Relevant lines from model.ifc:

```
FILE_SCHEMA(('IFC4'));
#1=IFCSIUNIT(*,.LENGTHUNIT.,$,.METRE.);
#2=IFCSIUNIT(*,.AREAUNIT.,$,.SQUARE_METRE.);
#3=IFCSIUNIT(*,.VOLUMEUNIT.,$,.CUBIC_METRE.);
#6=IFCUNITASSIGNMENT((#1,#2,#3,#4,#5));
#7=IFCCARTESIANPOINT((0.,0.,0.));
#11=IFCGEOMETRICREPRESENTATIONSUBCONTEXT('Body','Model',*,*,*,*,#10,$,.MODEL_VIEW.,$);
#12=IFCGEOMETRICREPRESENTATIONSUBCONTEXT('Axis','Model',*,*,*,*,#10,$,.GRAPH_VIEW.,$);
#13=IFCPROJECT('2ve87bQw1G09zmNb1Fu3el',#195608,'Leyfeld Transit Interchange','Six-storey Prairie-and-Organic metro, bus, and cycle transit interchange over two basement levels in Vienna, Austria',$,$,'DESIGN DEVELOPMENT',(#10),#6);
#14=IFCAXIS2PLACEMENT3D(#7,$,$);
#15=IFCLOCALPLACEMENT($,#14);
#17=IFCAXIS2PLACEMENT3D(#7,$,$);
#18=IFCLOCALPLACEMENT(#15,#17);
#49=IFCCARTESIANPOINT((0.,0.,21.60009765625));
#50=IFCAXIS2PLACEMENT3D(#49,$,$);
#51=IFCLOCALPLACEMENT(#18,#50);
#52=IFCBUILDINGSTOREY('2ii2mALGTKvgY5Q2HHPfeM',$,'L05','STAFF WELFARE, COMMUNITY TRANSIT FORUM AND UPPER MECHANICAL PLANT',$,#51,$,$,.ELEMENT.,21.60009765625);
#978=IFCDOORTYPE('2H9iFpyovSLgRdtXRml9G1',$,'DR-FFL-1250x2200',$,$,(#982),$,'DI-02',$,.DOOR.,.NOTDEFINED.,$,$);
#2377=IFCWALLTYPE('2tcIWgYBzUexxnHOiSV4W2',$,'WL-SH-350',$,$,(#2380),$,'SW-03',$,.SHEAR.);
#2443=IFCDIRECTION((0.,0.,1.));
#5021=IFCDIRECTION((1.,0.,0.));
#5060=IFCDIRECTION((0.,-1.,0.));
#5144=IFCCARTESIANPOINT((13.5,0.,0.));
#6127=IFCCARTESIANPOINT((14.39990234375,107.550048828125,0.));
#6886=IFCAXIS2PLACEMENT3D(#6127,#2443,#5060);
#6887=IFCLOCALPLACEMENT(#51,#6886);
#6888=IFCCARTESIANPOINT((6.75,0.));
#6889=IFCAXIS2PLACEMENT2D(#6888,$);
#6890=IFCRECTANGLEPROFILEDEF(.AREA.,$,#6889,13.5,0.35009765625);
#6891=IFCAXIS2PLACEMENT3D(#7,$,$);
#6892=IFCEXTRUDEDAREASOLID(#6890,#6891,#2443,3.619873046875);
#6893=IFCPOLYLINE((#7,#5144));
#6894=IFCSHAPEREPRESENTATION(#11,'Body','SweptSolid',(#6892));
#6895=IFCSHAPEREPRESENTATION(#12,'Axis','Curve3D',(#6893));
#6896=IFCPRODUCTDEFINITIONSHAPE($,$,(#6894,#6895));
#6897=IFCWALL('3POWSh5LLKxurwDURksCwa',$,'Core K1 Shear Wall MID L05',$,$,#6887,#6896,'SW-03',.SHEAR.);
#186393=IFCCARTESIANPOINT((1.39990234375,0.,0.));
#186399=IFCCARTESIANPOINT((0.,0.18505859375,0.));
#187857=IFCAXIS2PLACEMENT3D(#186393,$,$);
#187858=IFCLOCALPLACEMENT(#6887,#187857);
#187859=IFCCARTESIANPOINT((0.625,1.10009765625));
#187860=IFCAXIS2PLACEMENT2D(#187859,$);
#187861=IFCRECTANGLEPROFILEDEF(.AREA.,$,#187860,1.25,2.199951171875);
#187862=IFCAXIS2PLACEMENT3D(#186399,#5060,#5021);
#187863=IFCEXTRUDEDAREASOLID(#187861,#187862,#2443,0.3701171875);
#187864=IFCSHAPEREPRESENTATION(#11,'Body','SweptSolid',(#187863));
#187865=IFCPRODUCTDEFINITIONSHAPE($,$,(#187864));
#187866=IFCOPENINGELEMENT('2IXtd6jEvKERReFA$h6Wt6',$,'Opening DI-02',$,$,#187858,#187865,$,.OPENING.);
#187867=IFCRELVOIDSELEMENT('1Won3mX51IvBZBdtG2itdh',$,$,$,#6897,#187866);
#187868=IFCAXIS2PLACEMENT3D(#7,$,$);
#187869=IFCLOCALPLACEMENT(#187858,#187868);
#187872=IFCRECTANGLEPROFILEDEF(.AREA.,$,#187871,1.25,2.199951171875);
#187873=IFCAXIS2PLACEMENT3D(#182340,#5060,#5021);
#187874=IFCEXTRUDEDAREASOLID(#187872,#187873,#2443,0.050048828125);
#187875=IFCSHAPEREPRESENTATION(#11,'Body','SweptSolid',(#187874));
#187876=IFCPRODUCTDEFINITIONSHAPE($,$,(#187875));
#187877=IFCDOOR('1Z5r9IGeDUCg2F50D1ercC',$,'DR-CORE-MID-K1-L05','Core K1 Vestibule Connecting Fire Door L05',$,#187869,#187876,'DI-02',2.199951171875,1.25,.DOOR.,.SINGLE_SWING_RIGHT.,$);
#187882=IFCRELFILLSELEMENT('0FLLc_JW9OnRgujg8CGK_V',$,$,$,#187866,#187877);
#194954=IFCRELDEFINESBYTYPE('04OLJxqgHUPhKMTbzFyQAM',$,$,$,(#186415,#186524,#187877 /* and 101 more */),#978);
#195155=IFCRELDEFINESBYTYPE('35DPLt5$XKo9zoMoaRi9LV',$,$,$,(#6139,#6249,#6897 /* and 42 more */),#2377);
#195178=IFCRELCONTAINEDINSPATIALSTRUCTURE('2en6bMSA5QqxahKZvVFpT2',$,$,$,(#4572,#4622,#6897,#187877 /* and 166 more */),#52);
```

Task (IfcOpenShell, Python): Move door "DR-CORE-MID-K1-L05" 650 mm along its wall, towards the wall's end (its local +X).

```python
import ifcopenshell
import ifcopenshell.api.geometry
import ifcopenshell.util.placement

model = ifcopenshell.open("model.ifc")

door = model.by_guid("1Z5r9IGeDUCg2F50D1ercC")
opening = door.FillsVoids[0].RelatingOpeningElement
wall = opening.VoidsElements[0].RelatingBuildingElement

wall_matrix = ifcopenshell.util.placement.get_local_placement(wall.ObjectPlacement)
shift = wall_matrix[:3, 0] * 0.65
before = ifcopenshell.util.placement.get_local_placement(door.ObjectPlacement)[:3, 3].copy()

# The door is placed relative to its opening, so it follows when the opening moves.
matrix = ifcopenshell.util.placement.get_local_placement(opening.ObjectPlacement)
matrix[:3, 3] += shift
ifcopenshell.api.geometry.edit_object_placement(
    model, product=opening, matrix=matrix, is_si=False, should_transform_children=True
)

after = ifcopenshell.util.placement.get_local_placement(door.ObjectPlacement)[:3, 3]
print("door moved by", (after - before).round(3) + 0.0)

model.write("model_v2.ifc")
```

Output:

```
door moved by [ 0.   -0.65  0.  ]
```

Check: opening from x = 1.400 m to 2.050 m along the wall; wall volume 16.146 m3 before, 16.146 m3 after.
